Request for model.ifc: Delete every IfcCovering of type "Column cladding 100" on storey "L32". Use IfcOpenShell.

First a look at what the model holds.

```python
import ifcopenshell
import ifcopenshell.util.element

model = ifcopenshell.open("model.ifc")
print(model.schema)
storey = next(s for s in model.by_type("IfcBuildingStorey") if s.Name == "L32")
coverings = [e for e in ifcopenshell.util.element.get_decomposition(storey) if e.is_a("IfcCovering")]
seen = {}
for e in coverings:
    element_type = ifcopenshell.util.element.get_type(e)
    name = element_type.Name if element_type not in (None, e) else None
    seen[name] = seen.get(name, 0) + 1
for name, count in sorted(seen.items(), key=str):
    print(count, "x", name)
```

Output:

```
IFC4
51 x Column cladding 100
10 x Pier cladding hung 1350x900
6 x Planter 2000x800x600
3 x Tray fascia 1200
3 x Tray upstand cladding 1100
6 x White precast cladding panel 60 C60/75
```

```python
import ifcopenshell
import ifcopenshell.api.root
import ifcopenshell.util.element

model = ifcopenshell.open("model.ifc")

storey = next(s for s in model.by_type("IfcBuildingStorey") if s.Name == "L32")
coverings = [e for e in ifcopenshell.util.element.get_decomposition(storey) if e.is_a("IfcCovering")]
targets = [e for e in coverings if (t := ifcopenshell.util.element.get_type(e)) not in (None, e) and t.Name == "Column cladding 100"]

for e in targets:
    ifcopenshell.api.root.remove_product(model, product=e)
print(len(targets), "removed")

model.write("model_rev.ifc")
```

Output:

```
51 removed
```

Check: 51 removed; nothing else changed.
